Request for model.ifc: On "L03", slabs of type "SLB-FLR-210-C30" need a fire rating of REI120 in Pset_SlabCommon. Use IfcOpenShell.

First a look at what the model holds.

```python
import ifcopenshell
import ifcopenshell.util.element

model = ifcopenshell.open("model.ifc")
print(model.schema)
storey = next(s for s in model.by_type("IfcBuildingStorey") if s.Name == "L03")
slabs = [e for e in ifcopenshell.util.element.get_decomposition(storey) if e.is_a("IfcSlab")]
seen = {}
for e in slabs:
    element_type = ifcopenshell.util.element.get_type(e)
    key = (element_type.Name if element_type != e and element_type else None, ifcopenshell.util.element.get_pset(e, "Pset_SlabCommon", "FireRating"))
    seen[key] = seen.get(key, 0) + 1
for (name, value), count in sorted(seen.items(), key=str):
    print(count, "x", name, "|", value)
```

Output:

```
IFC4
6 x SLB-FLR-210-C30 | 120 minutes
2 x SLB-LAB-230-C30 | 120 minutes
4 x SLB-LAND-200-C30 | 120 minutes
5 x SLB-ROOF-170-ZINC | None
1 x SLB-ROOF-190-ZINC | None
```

```python
import ifcopenshell
import ifcopenshell.api.pset
import ifcopenshell.util.element

model = ifcopenshell.open("model.ifc")

storey = next(s for s in model.by_type("IfcBuildingStorey") if s.Name == "L03")
slabs = [e for e in ifcopenshell.util.element.get_decomposition(storey) if e.is_a("IfcSlab")]

count = 0
for e in slabs:
    element_type = ifcopenshell.util.element.get_type(e)
    if element_type in (None, e) or element_type.Name != "SLB-FLR-210-C30":
        continue
    # add_pset returns the element's existing set when there is one.
    pset = ifcopenshell.api.pset.add_pset(model, product=e, name="Pset_SlabCommon")
    ifcopenshell.api.pset.edit_pset(model, pset=pset, properties={"FireRating": "REI120"})
    count += 1

print(count, "slabs updated")

model.write("model_edited.ifc")
```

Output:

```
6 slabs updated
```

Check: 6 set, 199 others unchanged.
